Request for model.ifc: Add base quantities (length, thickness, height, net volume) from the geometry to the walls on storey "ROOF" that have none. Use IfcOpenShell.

First a look at what the model holds.

```python
import ifcopenshell
import ifcopenshell.util.element
import ifcopenshell.util.unit

model = ifcopenshell.open("model.ifc")
print(model.schema)
for unit_type in ("LENGTHUNIT", "AREAUNIT", "VOLUMEUNIT"):
    print(unit_type, ifcopenshell.util.unit.calculate_unit_scale(model, unit_type))
storey = next(s for s in model.by_type("IfcBuildingStorey") if s.Name == "ROOF")
walls = [e for e in ifcopenshell.util.element.get_decomposition(storey) if e.is_a("IfcWall")]
for e in sorted(walls, key=lambda e: e.id()):
    print(e.id(), e.is_a(), e.Name, list(ifcopenshell.util.element.get_psets(e, qtos_only=True)), sep=" | ")
```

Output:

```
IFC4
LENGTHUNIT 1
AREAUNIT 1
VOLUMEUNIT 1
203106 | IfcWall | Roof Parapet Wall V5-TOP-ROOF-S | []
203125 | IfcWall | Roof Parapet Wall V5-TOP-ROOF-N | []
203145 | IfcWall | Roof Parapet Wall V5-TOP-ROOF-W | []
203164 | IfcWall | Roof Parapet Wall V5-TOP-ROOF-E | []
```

```python
import ifcopenshell
import ifcopenshell.api.pset
import ifcopenshell.geom
import ifcopenshell.util.element
import ifcopenshell.util.shape
import ifcopenshell.util.unit

model = ifcopenshell.open("model.ifc")
unit_scale = ifcopenshell.util.unit.calculate_unit_scale(model)
volume_scale = ifcopenshell.util.unit.calculate_unit_scale(model, "VOLUMEUNIT")
settings = ifcopenshell.geom.settings()

storey = next(s for s in model.by_type("IfcBuildingStorey") if s.Name == "ROOF")
walls = [e for e in ifcopenshell.util.element.get_decomposition(storey) if e.is_a("IfcWall")]

for e in sorted(walls, key=lambda e: e.id()):
    if ifcopenshell.util.element.get_psets(e, qtos_only=True, should_inherit=False):
        continue
    # Geometry comes back in metres, in the element's own axes.
    shape = ifcopenshell.geom.create_shape(settings, e)
    values = {
        "Length": ifcopenshell.util.shape.get_x(shape.geometry) / unit_scale,
        "Width": ifcopenshell.util.shape.get_y(shape.geometry) / unit_scale,
        "Height": ifcopenshell.util.shape.get_z(shape.geometry) / unit_scale,
        "NetVolume": ifcopenshell.util.shape.get_volume(shape.geometry) / volume_scale,
    }
    qto = ifcopenshell.api.pset.add_qto(model, product=e, name="Qto_WallBaseQuantities")
    ifcopenshell.api.pset.edit_qto(model, qto=qto, properties=values)
    print(e.id(), {k: round(v, 3) for k, v in values.items()})

model.write("model_updated.ifc")
```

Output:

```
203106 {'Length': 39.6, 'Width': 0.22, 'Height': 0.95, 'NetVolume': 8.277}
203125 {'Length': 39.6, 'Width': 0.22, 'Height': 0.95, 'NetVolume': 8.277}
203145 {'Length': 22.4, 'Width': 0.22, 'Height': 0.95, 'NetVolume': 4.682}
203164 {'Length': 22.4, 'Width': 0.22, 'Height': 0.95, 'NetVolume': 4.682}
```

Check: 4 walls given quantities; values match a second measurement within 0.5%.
